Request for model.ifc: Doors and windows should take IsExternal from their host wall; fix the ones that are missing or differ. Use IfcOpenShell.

First a look at what the model holds.

```python
import ifcopenshell
import ifcopenshell.util.element

model = ifcopenshell.open("model.ifc")
print(model.schema)
seen = {}
for e in model.by_type("IfcDoor") + model.by_type("IfcWindow"):
    if not e.FillsVoids:
        continue
    host = e.FillsVoids[0].RelatingOpeningElement.VoidsElements[0].RelatingBuildingElement
    own = ifcopenshell.util.element.get_pset(e, f"Pset_{e.is_a()[3:].removesuffix('StandardCase')}Common", "IsExternal")
    wall = ifcopenshell.util.element.get_pset(host, "Pset_WallCommon", "IsExternal")
    seen[e.is_a(), own, wall] = seen.get((e.is_a(), own, wall), 0) + 1
for (cls, own, wall), count in sorted(seen.items(), key=str):
    print(count, cls, "IsExternal:", own, "| host wall:", wall)
```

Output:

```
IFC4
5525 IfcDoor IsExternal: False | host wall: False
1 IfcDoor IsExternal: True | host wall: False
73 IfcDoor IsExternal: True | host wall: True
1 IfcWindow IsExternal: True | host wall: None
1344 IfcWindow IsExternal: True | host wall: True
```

```python
import ifcopenshell
import ifcopenshell.api.pset
import ifcopenshell.util.element

model = ifcopenshell.open("model.ifc")

count = 0
for ifc_class, pset_name in (("IfcDoor", "Pset_DoorCommon"), ("IfcWindow", "Pset_WindowCommon")):
    for e in model.by_type(ifc_class):
        if not e.FillsVoids:
            continue
        host = e.FillsVoids[0].RelatingOpeningElement.VoidsElements[0].RelatingBuildingElement
        external = ifcopenshell.util.element.get_pset(host, "Pset_WallCommon", "IsExternal")
        if external is None or ifcopenshell.util.element.get_pset(e, pset_name, "IsExternal") == external:
            continue
        pset = ifcopenshell.api.pset.add_pset(model, product=e, name=pset_name)
        ifcopenshell.api.pset.edit_pset(model, pset=pset, properties={"IsExternal": external})
        count += 1

print(count, "updated")

model.write("model-out.ifc")
```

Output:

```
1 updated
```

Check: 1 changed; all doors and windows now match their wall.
